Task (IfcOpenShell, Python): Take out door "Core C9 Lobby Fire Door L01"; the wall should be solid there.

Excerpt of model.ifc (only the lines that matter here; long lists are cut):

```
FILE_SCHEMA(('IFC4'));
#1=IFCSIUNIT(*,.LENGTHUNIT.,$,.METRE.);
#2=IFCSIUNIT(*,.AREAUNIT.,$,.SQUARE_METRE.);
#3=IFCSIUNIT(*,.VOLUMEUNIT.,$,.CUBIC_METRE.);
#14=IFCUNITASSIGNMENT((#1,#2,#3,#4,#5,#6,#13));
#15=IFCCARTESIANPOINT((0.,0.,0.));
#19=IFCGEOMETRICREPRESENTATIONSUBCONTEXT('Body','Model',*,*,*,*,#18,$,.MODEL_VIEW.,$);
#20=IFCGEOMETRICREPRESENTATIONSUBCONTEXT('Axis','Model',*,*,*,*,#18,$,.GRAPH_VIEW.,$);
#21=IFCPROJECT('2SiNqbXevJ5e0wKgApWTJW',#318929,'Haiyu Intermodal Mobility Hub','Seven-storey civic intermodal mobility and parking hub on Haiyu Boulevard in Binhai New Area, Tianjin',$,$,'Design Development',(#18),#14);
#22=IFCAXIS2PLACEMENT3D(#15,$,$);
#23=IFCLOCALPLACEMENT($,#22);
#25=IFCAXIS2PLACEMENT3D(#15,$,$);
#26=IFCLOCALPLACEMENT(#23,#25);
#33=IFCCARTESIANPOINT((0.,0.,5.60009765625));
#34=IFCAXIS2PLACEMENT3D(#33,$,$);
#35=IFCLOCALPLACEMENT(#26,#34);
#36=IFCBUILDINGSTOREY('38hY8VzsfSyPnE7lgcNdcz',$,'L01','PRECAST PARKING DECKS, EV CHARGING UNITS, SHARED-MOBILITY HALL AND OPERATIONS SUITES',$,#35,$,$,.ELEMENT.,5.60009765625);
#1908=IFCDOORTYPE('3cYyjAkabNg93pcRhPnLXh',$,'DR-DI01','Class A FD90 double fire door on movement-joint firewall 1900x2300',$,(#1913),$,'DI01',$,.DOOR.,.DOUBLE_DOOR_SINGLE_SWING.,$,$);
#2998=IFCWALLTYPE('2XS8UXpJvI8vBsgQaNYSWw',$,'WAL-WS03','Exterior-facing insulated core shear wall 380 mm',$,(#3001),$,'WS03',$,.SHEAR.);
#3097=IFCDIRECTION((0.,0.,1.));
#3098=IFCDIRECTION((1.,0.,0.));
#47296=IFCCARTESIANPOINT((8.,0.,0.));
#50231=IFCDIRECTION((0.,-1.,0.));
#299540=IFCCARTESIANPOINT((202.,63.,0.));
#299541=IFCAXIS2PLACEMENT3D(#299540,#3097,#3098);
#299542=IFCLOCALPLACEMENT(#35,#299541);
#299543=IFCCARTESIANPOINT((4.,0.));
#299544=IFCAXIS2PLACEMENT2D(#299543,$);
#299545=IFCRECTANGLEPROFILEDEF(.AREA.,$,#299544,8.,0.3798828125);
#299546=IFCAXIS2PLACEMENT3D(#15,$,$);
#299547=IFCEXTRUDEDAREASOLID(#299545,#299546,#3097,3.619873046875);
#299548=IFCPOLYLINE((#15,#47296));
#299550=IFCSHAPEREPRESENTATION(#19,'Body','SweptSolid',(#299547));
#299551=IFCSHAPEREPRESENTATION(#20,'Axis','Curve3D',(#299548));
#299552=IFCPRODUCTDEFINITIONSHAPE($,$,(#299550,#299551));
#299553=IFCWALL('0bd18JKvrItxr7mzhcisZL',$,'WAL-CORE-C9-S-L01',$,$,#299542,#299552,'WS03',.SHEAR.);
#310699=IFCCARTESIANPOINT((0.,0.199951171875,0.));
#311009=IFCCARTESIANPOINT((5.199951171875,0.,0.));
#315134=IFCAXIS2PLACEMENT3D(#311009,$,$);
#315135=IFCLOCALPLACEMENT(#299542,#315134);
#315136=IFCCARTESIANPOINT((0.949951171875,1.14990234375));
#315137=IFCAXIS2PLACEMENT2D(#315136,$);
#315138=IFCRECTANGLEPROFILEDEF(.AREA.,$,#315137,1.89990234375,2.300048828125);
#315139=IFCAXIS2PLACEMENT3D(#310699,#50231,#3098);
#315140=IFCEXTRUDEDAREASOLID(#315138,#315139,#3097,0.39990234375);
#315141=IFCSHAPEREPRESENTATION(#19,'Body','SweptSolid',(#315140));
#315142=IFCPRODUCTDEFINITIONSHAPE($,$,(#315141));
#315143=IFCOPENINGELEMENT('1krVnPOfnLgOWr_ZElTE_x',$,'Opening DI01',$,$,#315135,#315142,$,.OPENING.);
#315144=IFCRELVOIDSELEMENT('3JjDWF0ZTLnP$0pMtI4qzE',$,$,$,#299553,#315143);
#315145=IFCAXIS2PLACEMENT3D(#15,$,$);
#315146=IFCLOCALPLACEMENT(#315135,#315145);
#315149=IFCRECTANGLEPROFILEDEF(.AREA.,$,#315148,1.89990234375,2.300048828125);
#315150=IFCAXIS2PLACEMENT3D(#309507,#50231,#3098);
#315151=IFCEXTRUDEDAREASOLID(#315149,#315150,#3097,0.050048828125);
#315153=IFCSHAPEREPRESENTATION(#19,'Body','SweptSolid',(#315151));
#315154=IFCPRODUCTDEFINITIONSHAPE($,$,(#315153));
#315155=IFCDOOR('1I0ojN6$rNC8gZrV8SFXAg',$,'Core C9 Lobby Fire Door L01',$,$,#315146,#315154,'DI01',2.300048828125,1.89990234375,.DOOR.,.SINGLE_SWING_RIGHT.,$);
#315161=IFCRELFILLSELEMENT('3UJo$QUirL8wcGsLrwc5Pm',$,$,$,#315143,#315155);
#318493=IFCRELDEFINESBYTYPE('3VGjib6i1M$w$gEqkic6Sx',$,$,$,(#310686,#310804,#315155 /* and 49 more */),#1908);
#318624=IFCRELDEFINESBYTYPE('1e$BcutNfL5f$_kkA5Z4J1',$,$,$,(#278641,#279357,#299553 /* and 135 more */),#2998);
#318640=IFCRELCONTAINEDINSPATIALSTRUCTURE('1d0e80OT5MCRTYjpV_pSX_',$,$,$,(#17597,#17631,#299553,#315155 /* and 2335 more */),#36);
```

```python
import ifcopenshell
import ifcopenshell.api.feature
import ifcopenshell.api.root
import ifcopenshell.geom
import ifcopenshell.util.shape

model = ifcopenshell.open("model.ifc")
settings = ifcopenshell.geom.settings()


def volume(element):
    """Net volume in cubic metres, openings subtracted."""
    shape = ifcopenshell.geom.create_shape(settings, element)
    return ifcopenshell.util.shape.get_volume(shape.geometry)


door = model.by_guid("1I0ojN6$rNC8gZrV8SFXAg")
opening = door.FillsVoids[0].RelatingOpeningElement
wall = opening.VoidsElements[0].RelatingBuildingElement
before = volume(wall)

ifcopenshell.api.root.remove_product(model, product=door)
ifcopenshell.api.feature.remove_feature(model, feature=opening)

after = volume(wall)

print(f"wall volume {before:.3f} -> {after:.3f} m3")

model.write("model_updated.ifc")
```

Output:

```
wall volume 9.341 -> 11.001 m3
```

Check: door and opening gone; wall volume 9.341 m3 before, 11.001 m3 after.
